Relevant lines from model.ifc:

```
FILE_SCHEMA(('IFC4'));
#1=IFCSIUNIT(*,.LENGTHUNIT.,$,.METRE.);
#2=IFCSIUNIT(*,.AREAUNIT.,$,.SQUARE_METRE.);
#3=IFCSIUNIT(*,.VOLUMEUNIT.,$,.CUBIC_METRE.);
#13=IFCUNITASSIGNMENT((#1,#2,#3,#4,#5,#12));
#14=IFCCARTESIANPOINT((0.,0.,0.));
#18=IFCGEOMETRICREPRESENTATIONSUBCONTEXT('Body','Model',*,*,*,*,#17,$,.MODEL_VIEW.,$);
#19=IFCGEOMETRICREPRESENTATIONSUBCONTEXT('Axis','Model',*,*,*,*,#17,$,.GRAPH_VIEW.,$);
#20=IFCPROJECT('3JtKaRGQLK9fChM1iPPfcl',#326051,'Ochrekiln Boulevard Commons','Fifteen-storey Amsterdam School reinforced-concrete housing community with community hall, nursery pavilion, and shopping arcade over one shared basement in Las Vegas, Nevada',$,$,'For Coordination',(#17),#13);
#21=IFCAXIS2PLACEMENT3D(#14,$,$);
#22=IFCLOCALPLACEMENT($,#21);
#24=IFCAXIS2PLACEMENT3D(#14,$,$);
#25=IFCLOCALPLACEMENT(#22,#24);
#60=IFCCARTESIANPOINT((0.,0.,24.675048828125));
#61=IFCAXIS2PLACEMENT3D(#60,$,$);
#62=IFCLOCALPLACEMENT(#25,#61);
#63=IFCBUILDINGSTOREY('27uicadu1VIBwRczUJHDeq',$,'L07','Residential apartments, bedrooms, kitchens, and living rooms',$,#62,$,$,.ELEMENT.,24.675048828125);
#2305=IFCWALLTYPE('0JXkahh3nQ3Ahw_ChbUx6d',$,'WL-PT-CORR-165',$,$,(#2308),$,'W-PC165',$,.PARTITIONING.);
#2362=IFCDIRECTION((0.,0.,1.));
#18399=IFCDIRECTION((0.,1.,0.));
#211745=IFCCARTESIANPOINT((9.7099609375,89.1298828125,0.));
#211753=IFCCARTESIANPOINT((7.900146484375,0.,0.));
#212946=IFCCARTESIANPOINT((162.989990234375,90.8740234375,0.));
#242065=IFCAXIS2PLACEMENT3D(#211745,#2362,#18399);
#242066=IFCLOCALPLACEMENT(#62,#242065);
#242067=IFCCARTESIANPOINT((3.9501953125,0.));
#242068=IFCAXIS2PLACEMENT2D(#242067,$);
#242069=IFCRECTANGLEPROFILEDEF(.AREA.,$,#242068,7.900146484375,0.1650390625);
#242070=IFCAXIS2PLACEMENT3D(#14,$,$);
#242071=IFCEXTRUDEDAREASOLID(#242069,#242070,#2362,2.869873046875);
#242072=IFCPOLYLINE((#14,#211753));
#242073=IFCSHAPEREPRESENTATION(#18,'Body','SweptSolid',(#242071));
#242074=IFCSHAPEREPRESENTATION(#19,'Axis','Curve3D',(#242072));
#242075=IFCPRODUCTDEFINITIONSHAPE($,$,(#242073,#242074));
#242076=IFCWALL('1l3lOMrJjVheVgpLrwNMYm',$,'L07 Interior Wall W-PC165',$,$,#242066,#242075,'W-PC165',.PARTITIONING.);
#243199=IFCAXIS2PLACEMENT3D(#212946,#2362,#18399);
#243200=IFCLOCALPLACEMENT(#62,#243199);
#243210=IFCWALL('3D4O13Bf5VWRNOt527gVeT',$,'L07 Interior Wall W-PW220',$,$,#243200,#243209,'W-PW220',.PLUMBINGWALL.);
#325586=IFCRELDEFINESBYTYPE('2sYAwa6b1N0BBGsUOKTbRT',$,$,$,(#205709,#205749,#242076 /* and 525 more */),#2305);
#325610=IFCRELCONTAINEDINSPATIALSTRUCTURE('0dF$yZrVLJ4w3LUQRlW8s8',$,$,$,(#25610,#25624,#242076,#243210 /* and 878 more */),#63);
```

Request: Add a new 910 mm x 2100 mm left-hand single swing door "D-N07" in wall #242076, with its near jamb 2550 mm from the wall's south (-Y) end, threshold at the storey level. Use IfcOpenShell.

```python
import numpy as np
import ifcopenshell
import ifcopenshell.api.feature
import ifcopenshell.api.geometry
import ifcopenshell.api.root
import ifcopenshell.api.spatial
import ifcopenshell.geom
import ifcopenshell.util.element
import ifcopenshell.util.placement
import ifcopenshell.util.representation
import ifcopenshell.util.shape
import ifcopenshell.util.unit

model = ifcopenshell.open("model.ifc")
unit_scale = ifcopenshell.util.unit.calculate_unit_scale(model)
settings = ifcopenshell.geom.settings()


def volume(element):
    """Net volume in cubic metres, openings subtracted."""
    shape = ifcopenshell.geom.create_shape(settings, element)
    return ifcopenshell.util.shape.get_volume(shape.geometry)


wall = model.by_id(242076)
storey = ifcopenshell.util.element.get_container(wall, ifc_class="IfcBuildingStorey")
context = ifcopenshell.util.representation.get_context(model, "Model", "Body", "MODEL_VIEW")
before = volume(wall)

width, height, from_end, sill = 0.91, 2.1, 2.55, 0.0  # metres

# The wall runs along its own X axis, and the end named is its -X end.
wall_shape = ifcopenshell.geom.create_shape(settings, wall)
x, y, z = ifcopenshell.util.shape.get_vertices(wall_shape.geometry).T
start = x.min() + from_end
face, thickness = float(y.min()), float(y.max() - y.min())
wall_matrix = ifcopenshell.util.placement.get_local_placement(wall.ObjectPlacement)
level = ifcopenshell.util.placement.get_local_placement(storey.ObjectPlacement)[2, 3]


def in_wall(x, y):
    """Placement at x, y metres in the wall's axes, at sill height."""
    matrix = wall_matrix.copy()
    matrix[:, 3] = wall_matrix @ np.array([x / unit_scale, y / unit_scale, 0.0, 1.0])
    matrix[2, 3] = level + sill / unit_scale
    return matrix


# Opening: a box that overshoots both wall faces by 50 mm.
opening = ifcopenshell.api.root.create_entity(model, ifc_class="IfcOpeningElement", predefined_type="OPENING")
box = ifcopenshell.api.geometry.add_wall_representation(
    model, context=context, length=width, height=height, thickness=thickness + 0.1
)
ifcopenshell.api.geometry.assign_representation(model, product=opening, representation=box)
ifcopenshell.api.geometry.edit_object_placement(model, product=opening, matrix=in_wall(start, face - 0.05), is_si=False)
ifcopenshell.api.feature.add_feature(model, feature=opening, element=wall)

door = ifcopenshell.api.root.create_entity(model, ifc_class="IfcDoor", name="D-N07", predefined_type="DOOR")
door.OverallWidth, door.OverallHeight = width / unit_scale, height / unit_scale
door.OperationType = "SINGLE_SWING_LEFT"
body = ifcopenshell.api.geometry.add_door_representation(
    model,
    context=context,
    overall_width=door.OverallWidth,
    overall_height=door.OverallHeight,
    operation_type="SINGLE_SWING_LEFT",
    lining_properties={"LiningDepth": thickness / unit_scale, "ThresholdDepth": thickness / unit_scale},
)
ifcopenshell.api.geometry.assign_representation(model, product=door, representation=body)
ifcopenshell.api.spatial.assign_container(model, products=[door], relating_structure=storey)
ifcopenshell.api.feature.add_filling(model, opening=opening, element=door)

# The lining spans the wall, so the door starts at the wall face.
ifcopenshell.api.geometry.edit_object_placement(model, product=door, matrix=in_wall(start, face), is_si=False)

after = volume(wall)

print(f"wall volume {before:.3f} -> {after:.3f} m3")

model.write("model_updated.ifc")
```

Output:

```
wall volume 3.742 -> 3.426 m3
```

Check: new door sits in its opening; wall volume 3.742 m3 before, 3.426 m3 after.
